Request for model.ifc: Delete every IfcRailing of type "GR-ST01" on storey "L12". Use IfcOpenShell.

First a look at what the model holds.

```python
import ifcopenshell
import ifcopenshell.util.element

model = ifcopenshell.open("model.ifc")
print(model.schema)
storey = next(s for s in model.by_type("IfcBuildingStorey") if s.Name == "L12")
railings = [e for e in ifcopenshell.util.element.get_decomposition(storey) if e.is_a("IfcRailing")]
seen = {}
for e in railings:
    element_type = ifcopenshell.util.element.get_type(e)
    name = element_type.Name if element_type not in (None, e) else None
    seen[name] = seen.get(name, 0) + 1
for name, count in sorted(seen.items(), key=str):
    print(count, "x", name)
```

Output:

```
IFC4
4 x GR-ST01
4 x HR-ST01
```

```python
import ifcopenshell
import ifcopenshell.api.root
import ifcopenshell.util.element

model = ifcopenshell.open("model.ifc")

storey = next(s for s in model.by_type("IfcBuildingStorey") if s.Name == "L12")
railings = [e for e in ifcopenshell.util.element.get_decomposition(storey) if e.is_a("IfcRailing")]
targets = [e for e in railings if (t := ifcopenshell.util.element.get_type(e)) not in (None, e) and t.Name == "GR-ST01"]

for e in targets:
    ifcopenshell.api.root.remove_product(model, product=e)
print(len(targets), "removed")

model.write("model_edited.ifc")
```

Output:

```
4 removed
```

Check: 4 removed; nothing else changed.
